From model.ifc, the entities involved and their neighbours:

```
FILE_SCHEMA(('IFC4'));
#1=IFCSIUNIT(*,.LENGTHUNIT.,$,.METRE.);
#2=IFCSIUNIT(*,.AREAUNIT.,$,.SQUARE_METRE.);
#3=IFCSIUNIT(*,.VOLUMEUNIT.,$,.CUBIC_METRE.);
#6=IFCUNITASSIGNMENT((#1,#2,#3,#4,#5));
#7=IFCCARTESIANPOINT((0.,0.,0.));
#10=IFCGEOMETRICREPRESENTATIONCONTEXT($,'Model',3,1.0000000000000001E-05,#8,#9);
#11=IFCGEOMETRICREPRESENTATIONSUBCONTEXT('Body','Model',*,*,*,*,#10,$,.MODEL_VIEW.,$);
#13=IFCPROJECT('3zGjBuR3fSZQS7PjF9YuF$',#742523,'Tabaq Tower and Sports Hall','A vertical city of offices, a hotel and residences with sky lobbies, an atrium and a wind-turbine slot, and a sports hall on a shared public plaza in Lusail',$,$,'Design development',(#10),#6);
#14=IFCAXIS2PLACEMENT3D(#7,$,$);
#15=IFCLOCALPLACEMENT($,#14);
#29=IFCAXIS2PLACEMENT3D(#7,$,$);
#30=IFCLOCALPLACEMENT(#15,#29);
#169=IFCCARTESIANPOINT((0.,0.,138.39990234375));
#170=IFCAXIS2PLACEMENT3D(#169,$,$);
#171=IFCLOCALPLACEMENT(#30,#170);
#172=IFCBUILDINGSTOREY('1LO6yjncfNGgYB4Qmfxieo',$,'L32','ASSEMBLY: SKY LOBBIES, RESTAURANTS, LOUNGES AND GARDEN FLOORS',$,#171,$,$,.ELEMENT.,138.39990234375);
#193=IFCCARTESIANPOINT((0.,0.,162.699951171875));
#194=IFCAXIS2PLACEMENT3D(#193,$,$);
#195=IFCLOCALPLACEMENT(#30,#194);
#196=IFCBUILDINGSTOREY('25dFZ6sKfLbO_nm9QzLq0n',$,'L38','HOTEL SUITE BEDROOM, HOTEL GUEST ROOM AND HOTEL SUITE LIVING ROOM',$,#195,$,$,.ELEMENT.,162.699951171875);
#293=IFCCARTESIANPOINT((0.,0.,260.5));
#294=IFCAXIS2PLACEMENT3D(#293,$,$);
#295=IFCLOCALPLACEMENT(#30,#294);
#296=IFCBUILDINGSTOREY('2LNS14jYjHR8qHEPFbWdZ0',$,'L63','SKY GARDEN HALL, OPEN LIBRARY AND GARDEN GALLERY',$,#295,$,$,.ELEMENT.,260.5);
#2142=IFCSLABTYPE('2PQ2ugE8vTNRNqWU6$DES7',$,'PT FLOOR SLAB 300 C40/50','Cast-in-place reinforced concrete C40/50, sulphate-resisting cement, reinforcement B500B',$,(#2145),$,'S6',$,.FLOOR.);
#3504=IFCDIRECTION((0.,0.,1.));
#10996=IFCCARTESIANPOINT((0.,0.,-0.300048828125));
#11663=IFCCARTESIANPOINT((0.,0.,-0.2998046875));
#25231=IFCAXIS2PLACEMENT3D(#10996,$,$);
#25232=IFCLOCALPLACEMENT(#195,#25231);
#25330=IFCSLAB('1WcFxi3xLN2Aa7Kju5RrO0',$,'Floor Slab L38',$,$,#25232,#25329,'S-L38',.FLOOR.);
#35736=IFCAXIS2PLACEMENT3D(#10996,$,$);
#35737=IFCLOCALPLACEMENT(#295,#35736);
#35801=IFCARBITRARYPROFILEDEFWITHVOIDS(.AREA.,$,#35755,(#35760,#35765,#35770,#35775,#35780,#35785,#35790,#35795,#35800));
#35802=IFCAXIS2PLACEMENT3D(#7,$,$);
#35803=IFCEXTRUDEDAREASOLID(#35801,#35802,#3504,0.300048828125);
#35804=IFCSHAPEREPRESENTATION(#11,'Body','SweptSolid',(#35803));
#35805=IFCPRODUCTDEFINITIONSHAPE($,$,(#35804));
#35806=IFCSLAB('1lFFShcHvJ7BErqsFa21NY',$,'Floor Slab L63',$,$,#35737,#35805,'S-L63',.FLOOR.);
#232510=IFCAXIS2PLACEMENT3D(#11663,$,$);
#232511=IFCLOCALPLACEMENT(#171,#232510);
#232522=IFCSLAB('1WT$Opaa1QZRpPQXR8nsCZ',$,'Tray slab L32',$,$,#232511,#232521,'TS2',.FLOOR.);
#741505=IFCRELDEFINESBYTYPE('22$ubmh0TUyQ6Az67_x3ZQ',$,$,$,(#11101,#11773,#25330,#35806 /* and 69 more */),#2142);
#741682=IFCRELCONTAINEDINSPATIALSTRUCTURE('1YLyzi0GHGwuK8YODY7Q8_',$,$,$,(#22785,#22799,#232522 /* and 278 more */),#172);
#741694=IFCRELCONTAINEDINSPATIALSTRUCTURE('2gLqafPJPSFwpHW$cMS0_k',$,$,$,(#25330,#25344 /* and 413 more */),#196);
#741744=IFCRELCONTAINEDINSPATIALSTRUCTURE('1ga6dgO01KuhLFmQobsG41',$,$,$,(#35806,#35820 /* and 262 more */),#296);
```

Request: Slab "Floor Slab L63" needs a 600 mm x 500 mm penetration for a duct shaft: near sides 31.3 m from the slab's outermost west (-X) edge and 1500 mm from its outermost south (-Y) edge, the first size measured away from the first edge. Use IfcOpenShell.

```python
import numpy as np
import ifcopenshell
import ifcopenshell.api.feature
import ifcopenshell.api.geometry
import ifcopenshell.api.root
import ifcopenshell.geom
import ifcopenshell.util.placement
import ifcopenshell.util.representation
import ifcopenshell.util.shape
import ifcopenshell.util.unit

model = ifcopenshell.open("model.ifc")
unit_scale = ifcopenshell.util.unit.calculate_unit_scale(model)
settings = ifcopenshell.geom.settings()


def volume(element):
    """Net volume in cubic metres, openings subtracted."""
    shape = ifcopenshell.geom.create_shape(settings, element)
    return ifcopenshell.util.shape.get_volume(shape.geometry)


slab = model.by_guid("1lFFShcHvJ7BErqsFa21NY")
before = volume(slab)

# Extent in the slab's own axes, in metres. The edges named are its -X and -Y sides.
slab_shape = ifcopenshell.geom.create_shape(settings, slab)
vertices = ifcopenshell.util.shape.get_vertices(slab_shape.geometry)
x_min, y_min, bottom = vertices.min(axis=0)
top = vertices[:, 2].max()

opening = ifcopenshell.api.root.create_entity(model, ifc_class="IfcOpeningElement", name="Duct shaft opening", predefined_type="OPENING")
context = ifcopenshell.util.representation.get_context(model, "Model", "Body", "MODEL_VIEW")
width, depth = 0.6, 0.5
outline = [(0.0, 0.0), (width, 0.0), (width, depth), (0.0, depth), (0.0, 0.0)]
# Overshoot both faces by 50 mm so the cut is clean.
shape = ifcopenshell.api.geometry.add_slab_representation(
    model, context=context, depth=top - bottom + 0.1, polyline=outline
)
ifcopenshell.api.geometry.assign_representation(model, product=opening, representation=shape)

matrix = ifcopenshell.util.placement.get_local_placement(slab.ObjectPlacement)
matrix[:, 3] = matrix @ np.append(np.array([x_min + 31.3, y_min + 1.5, bottom - 0.05]) / unit_scale, 1.0)
ifcopenshell.api.geometry.edit_object_placement(model, product=opening, matrix=matrix, is_si=False)
ifcopenshell.api.feature.add_feature(model, feature=opening, element=slab)

after = volume(slab)

print(f"slab volume {before:.3f} -> {after:.3f} m3")

model.write("model_v2.ifc")
```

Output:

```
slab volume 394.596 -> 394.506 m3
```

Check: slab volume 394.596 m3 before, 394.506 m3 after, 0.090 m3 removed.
